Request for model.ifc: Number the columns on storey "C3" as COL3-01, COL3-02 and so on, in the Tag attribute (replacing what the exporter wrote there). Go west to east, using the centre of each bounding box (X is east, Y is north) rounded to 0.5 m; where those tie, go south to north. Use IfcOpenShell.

First a look at what the model holds.

```python
import ifcopenshell
import ifcopenshell.util.element
import ifcopenshell.util.placement

model = ifcopenshell.open("model.ifc")
print(model.schema)
storey = next(s for s in model.by_type("IfcBuildingStorey") if s.Name == "C3")
columns = [e for e in ifcopenshell.util.element.get_decomposition(storey) if e.is_a("IfcColumn")]
for e in sorted(columns, key=lambda e: e.id()):
    origin = ifcopenshell.util.placement.get_local_placement(e.ObjectPlacement)[:3, 3]
    print(e.id(), e.Tag, e.Name, origin.round(2) + 0.0, sep=" | ")
```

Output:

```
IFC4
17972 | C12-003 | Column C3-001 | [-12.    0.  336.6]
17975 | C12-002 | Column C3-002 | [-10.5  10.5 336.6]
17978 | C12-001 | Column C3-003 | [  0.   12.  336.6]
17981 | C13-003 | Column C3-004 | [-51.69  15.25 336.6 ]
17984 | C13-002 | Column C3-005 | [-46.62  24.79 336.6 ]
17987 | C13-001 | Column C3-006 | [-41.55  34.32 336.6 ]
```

```python
import ifcopenshell
import ifcopenshell.geom
import ifcopenshell.util.element
import ifcopenshell.util.shape

model = ifcopenshell.open("model.ifc")
settings = ifcopenshell.geom.settings()
settings.set("use-world-coords", True)


def centre(element):
    shape = ifcopenshell.geom.create_shape(settings, element)
    return ifcopenshell.util.shape.get_bbox_centroid(shape.geometry)


storey = next(s for s in model.by_type("IfcBuildingStorey") if s.Name == "C3")
columns = [e for e in ifcopenshell.util.element.get_decomposition(storey) if e.is_a("IfcColumn")]

# Insertion points can sit at a corner or the storey origin, so sort by the geometry (in metres).
centres = {e: centre(e) for e in columns}
columns.sort(key=lambda e: (round(centres[e][0] / 0.5), centres[e][1]))

for i, e in enumerate(columns, start=1):
    number = f"COL3-{i:02d}"
    e.Tag = number
    print(e.id(), number)

model.write("model_updated.ifc")
```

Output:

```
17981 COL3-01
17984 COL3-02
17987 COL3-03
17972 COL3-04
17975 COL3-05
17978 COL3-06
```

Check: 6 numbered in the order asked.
